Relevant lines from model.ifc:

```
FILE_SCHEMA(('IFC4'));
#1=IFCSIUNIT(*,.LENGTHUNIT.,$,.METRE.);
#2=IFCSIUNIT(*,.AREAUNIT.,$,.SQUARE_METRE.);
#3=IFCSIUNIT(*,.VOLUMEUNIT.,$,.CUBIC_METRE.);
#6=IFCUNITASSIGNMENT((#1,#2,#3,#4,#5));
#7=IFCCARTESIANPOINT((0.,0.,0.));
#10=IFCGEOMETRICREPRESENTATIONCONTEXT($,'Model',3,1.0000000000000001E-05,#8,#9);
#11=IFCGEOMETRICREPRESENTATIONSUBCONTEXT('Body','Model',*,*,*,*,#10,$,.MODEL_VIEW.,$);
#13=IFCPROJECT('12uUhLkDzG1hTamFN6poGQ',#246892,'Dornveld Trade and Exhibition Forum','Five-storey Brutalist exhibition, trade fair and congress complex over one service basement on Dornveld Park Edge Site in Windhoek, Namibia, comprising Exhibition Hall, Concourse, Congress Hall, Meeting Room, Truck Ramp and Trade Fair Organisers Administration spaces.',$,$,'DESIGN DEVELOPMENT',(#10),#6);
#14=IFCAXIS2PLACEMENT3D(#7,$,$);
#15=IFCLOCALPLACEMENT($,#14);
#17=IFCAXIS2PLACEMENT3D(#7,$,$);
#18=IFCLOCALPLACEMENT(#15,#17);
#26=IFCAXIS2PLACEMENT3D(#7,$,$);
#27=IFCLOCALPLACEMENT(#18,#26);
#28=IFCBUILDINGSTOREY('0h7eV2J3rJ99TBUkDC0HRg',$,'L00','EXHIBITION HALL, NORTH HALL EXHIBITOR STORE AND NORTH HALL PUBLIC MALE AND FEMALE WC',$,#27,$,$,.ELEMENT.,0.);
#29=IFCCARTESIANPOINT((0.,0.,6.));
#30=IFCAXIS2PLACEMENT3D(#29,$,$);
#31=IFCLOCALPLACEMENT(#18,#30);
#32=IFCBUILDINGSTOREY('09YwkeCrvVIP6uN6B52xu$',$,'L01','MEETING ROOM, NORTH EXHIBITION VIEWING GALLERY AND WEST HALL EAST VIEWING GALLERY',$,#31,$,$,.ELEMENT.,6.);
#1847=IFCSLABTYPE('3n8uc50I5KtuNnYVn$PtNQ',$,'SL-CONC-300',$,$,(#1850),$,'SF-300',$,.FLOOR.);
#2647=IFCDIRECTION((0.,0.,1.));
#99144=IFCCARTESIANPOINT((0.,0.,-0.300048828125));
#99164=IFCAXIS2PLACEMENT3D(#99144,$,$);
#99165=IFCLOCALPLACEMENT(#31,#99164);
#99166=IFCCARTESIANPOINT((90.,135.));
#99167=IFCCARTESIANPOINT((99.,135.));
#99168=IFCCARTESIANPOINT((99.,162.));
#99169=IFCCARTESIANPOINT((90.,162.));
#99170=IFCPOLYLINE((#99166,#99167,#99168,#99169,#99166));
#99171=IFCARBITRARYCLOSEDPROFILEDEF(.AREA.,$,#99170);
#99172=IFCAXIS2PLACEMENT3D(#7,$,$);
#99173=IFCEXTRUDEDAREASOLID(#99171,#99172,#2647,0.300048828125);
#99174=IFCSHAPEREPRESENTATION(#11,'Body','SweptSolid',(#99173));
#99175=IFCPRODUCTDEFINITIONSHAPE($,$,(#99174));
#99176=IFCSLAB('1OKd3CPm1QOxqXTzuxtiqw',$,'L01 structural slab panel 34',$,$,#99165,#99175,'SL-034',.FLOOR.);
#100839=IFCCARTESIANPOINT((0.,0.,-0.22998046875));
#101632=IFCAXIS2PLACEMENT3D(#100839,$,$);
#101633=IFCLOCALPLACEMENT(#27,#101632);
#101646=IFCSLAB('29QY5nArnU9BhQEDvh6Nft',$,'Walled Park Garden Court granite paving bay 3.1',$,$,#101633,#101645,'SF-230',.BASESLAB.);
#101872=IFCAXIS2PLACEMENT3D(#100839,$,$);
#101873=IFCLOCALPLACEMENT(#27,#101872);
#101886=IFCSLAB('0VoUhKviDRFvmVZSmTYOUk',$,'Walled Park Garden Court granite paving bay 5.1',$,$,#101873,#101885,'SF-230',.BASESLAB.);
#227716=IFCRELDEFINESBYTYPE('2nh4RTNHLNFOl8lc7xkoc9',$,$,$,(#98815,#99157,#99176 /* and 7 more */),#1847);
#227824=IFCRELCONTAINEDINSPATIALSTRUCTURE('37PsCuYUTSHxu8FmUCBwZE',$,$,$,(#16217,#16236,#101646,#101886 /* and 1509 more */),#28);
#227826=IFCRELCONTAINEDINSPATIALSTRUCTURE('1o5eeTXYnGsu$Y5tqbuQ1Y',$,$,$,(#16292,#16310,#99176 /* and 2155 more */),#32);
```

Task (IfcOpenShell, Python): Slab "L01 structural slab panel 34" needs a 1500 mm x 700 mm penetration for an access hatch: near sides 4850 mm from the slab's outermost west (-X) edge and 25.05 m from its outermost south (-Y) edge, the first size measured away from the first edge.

```python
import numpy as np
import ifcopenshell
import ifcopenshell.api.feature
import ifcopenshell.api.geometry
import ifcopenshell.api.root
import ifcopenshell.geom
import ifcopenshell.util.placement
import ifcopenshell.util.representation
import ifcopenshell.util.shape
import ifcopenshell.util.unit

model = ifcopenshell.open("model.ifc")
unit_scale = ifcopenshell.util.unit.calculate_unit_scale(model)
settings = ifcopenshell.geom.settings()


def volume(element):
    """Net volume in cubic metres, openings subtracted."""
    shape = ifcopenshell.geom.create_shape(settings, element)
    return ifcopenshell.util.shape.get_volume(shape.geometry)


slab = model.by_guid("1OKd3CPm1QOxqXTzuxtiqw")
before = volume(slab)

# Extent in the slab's own axes, in metres. The edges named are its -X and -Y sides.
slab_shape = ifcopenshell.geom.create_shape(settings, slab)
vertices = ifcopenshell.util.shape.get_vertices(slab_shape.geometry)
x_min, y_min, bottom = vertices.min(axis=0)
top = vertices[:, 2].max()

opening = ifcopenshell.api.root.create_entity(model, ifc_class="IfcOpeningElement", name="Access hatch opening", predefined_type="OPENING")
context = ifcopenshell.util.representation.get_context(model, "Model", "Body", "MODEL_VIEW")
width, depth = 1.5, 0.7
outline = [(0.0, 0.0), (width, 0.0), (width, depth), (0.0, depth), (0.0, 0.0)]
# Overshoot both faces by 50 mm so the cut is clean.
shape = ifcopenshell.api.geometry.add_slab_representation(
    model, context=context, depth=top - bottom + 0.1, polyline=outline
)
ifcopenshell.api.geometry.assign_representation(model, product=opening, representation=shape)

matrix = ifcopenshell.util.placement.get_local_placement(slab.ObjectPlacement)
matrix[:, 3] = matrix @ np.append(np.array([x_min + 4.85, y_min + 25.05, bottom - 0.05]) / unit_scale, 1.0)
ifcopenshell.api.geometry.edit_object_placement(model, product=opening, matrix=matrix, is_si=False)
ifcopenshell.api.feature.add_feature(model, feature=opening, element=slab)

after = volume(slab)

print(f"slab volume {before:.3f} -> {after:.3f} m3")

model.write("model_updated.ifc")
```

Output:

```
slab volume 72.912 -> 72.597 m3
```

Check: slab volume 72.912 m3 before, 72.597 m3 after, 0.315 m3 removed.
